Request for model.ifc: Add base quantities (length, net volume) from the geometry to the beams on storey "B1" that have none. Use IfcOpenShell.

First a look at what the model holds.

```python
import ifcopenshell
import ifcopenshell.util.element
import ifcopenshell.util.unit

model = ifcopenshell.open("model.ifc")
print(model.schema)
for unit_type in ("LENGTHUNIT", "AREAUNIT", "VOLUMEUNIT"):
    print(unit_type, ifcopenshell.util.unit.calculate_unit_scale(model, unit_type))
storey = next(s for s in model.by_type("IfcBuildingStorey") if s.Name == "B1")
beams = [e for e in ifcopenshell.util.element.get_decomposition(storey) if e.is_a("IfcBeam")]
for e in sorted(beams, key=lambda e: e.id()):
    print(e.id(), e.is_a(), e.Name, list(ifcopenshell.util.element.get_psets(e, qtos_only=True)), sep=" | ")
```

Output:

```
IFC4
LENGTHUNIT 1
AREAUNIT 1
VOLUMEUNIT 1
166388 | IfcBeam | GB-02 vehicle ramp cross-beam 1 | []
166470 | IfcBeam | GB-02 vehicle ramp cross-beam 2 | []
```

```python
import ifcopenshell
import ifcopenshell.api.pset
import ifcopenshell.geom
import ifcopenshell.util.element
import ifcopenshell.util.shape
import ifcopenshell.util.unit

model = ifcopenshell.open("model.ifc")
unit_scale = ifcopenshell.util.unit.calculate_unit_scale(model)
volume_scale = ifcopenshell.util.unit.calculate_unit_scale(model, "VOLUMEUNIT")
settings = ifcopenshell.geom.settings()

storey = next(s for s in model.by_type("IfcBuildingStorey") if s.Name == "B1")
beams = [e for e in ifcopenshell.util.element.get_decomposition(storey) if e.is_a("IfcBeam")]

for e in sorted(beams, key=lambda e: e.id()):
    if ifcopenshell.util.element.get_psets(e, qtos_only=True, should_inherit=False):
        continue
    # Geometry comes back in metres, in the element's own axes.
    shape = ifcopenshell.geom.create_shape(settings, e)
    values = {
        "Length": ifcopenshell.util.shape.get_max_xyz(shape.geometry) / unit_scale,
        "NetVolume": ifcopenshell.util.shape.get_volume(shape.geometry) / volume_scale,
    }
    qto = ifcopenshell.api.pset.add_qto(model, product=e, name="Qto_BeamBaseQuantities")
    ifcopenshell.api.pset.edit_qto(model, qto=qto, properties=values)
    print(e.id(), {k: round(v, 3) for k, v in values.items()})

model.write("model_rev.ifc")
```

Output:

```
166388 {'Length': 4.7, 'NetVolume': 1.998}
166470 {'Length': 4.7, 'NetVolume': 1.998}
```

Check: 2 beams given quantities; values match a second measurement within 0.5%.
